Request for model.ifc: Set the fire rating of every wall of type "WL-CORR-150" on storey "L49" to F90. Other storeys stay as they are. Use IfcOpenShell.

First a look at what the model holds.

```python
import ifcopenshell
import ifcopenshell.util.element

model = ifcopenshell.open("model.ifc")
print(model.schema)
storey = next(s for s in model.by_type("IfcBuildingStorey") if s.Name == "L49")
walls = [e for e in ifcopenshell.util.element.get_decomposition(storey) if e.is_a("IfcWall")]
seen = {}
for e in walls:
    element_type = ifcopenshell.util.element.get_type(e)
    key = (element_type.Name if element_type != e and element_type else None, ifcopenshell.util.element.get_pset(e, "Pset_WallCommon", "FireRating"))
    seen[key] = seen.get(key, 0) + 1
for (name, value), count in sorted(seen.items(), key=str):
    print(count, "x", name, "|", value)
```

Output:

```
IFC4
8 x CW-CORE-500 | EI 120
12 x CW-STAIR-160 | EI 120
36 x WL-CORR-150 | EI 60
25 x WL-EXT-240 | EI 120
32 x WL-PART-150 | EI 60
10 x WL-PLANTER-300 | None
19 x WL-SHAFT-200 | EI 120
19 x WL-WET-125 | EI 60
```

```python
import ifcopenshell
import ifcopenshell.api.pset
import ifcopenshell.util.element

model = ifcopenshell.open("model.ifc")

storey = next(s for s in model.by_type("IfcBuildingStorey") if s.Name == "L49")
walls = [e for e in ifcopenshell.util.element.get_decomposition(storey) if e.is_a("IfcWall")]

count = 0
for e in walls:
    element_type = ifcopenshell.util.element.get_type(e)
    if element_type in (None, e) or element_type.Name != "WL-CORR-150":
        continue
    found = ifcopenshell.util.element.get_pset(e, "Pset_WallCommon", should_inherit=False)
    if found:
        pset = model.by_id(found["id"])
        if len(ifcopenshell.util.element.get_elements_by_pset(pset)) > 1:
            pset = ifcopenshell.api.pset.unshare_pset(model, products=[e], pset=pset)[0]
    else:
        pset = ifcopenshell.api.pset.add_pset(model, product=e, name="Pset_WallCommon")
    ifcopenshell.api.pset.edit_pset(model, pset=pset, properties={"FireRating": "F90"})
    count += 1

print(count, "walls updated")

model.write("model-out.ifc")
```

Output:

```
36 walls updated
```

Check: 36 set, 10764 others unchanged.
